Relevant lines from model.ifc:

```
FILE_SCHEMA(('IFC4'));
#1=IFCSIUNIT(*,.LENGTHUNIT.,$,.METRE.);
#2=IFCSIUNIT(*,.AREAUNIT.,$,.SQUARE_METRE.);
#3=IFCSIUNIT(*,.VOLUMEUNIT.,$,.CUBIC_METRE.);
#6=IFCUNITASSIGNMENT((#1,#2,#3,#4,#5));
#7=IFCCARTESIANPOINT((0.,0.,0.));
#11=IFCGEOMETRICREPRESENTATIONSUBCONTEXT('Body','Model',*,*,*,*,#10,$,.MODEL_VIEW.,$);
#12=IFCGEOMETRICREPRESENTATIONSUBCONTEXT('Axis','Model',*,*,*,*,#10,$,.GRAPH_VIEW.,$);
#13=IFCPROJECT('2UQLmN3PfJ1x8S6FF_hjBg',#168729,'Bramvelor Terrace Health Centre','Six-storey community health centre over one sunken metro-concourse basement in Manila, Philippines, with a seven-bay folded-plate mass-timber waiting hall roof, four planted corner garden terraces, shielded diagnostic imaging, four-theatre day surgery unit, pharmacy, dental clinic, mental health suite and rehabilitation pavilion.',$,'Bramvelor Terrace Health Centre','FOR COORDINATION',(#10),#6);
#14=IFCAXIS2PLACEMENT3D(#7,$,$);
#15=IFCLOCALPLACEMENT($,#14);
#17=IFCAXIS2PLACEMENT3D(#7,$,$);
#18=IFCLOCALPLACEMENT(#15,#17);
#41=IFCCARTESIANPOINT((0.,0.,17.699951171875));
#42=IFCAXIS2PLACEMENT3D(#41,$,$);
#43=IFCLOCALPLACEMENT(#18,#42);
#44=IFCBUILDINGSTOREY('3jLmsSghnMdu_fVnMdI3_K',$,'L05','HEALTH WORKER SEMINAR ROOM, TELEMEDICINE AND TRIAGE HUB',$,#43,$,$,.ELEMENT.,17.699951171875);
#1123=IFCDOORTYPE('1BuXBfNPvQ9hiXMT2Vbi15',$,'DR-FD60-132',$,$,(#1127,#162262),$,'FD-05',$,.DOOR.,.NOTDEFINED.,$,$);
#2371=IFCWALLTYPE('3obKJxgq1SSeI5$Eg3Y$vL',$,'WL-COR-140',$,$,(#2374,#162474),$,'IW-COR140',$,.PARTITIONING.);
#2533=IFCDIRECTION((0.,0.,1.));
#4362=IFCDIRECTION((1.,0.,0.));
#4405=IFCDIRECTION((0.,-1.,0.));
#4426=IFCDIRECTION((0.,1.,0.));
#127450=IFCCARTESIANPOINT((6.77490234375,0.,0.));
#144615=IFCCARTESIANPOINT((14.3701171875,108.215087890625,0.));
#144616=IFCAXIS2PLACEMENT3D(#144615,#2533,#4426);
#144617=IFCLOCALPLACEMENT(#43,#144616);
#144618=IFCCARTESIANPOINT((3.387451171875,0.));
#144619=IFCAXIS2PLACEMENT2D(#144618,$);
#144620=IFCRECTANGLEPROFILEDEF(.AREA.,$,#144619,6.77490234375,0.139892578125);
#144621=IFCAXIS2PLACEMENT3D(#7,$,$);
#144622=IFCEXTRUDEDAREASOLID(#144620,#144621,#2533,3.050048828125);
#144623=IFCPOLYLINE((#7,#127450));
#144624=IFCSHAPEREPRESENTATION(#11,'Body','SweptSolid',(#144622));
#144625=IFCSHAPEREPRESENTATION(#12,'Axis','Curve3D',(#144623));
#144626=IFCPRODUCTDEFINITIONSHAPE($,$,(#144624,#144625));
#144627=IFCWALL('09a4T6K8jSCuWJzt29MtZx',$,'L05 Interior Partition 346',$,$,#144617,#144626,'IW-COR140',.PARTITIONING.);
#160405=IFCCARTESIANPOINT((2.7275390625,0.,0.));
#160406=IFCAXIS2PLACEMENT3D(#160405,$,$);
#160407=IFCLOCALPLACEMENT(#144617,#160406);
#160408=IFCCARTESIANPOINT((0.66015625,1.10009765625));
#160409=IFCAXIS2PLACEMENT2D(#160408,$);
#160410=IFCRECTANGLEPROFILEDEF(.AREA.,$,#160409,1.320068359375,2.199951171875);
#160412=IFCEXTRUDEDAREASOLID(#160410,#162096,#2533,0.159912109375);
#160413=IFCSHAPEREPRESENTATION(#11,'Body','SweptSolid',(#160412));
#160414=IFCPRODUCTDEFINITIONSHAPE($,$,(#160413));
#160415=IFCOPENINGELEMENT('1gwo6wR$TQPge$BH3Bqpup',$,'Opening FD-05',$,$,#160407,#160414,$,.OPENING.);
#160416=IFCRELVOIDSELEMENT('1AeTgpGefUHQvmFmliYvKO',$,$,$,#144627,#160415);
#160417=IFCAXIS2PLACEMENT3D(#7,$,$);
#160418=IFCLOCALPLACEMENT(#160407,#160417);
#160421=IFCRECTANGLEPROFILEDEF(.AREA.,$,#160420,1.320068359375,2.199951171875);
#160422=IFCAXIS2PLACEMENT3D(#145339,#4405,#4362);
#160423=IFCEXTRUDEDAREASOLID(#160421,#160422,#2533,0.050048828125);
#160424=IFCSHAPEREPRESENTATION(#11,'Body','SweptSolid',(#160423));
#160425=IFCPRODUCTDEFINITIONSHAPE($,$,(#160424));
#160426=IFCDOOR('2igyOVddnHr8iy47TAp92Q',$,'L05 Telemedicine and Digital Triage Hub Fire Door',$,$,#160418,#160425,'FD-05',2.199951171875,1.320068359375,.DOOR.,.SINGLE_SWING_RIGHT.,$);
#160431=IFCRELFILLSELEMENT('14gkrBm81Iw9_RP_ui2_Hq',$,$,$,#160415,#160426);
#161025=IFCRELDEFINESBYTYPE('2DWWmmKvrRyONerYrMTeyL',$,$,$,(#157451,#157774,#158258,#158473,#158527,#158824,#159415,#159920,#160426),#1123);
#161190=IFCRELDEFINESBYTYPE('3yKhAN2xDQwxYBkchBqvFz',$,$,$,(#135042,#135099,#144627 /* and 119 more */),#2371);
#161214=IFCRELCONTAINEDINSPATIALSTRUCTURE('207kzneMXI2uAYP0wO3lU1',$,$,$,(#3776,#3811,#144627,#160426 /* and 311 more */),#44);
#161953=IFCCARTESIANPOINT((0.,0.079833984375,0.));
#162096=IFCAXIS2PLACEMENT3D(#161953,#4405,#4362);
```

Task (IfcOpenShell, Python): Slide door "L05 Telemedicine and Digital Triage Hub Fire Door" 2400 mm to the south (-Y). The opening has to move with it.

```python
import ifcopenshell
import ifcopenshell.api.geometry
import ifcopenshell.util.placement

model = ifcopenshell.open("model.ifc")

door = model.by_guid("2igyOVddnHr8iy47TAp92Q")
opening = door.FillsVoids[0].RelatingOpeningElement
wall = opening.VoidsElements[0].RelatingBuildingElement

wall_matrix = ifcopenshell.util.placement.get_local_placement(wall.ObjectPlacement)
shift = wall_matrix[:3, 0] * -2.4
before = ifcopenshell.util.placement.get_local_placement(door.ObjectPlacement)[:3, 3].copy()

# The door is placed relative to its opening, so it follows when the opening moves.
matrix = ifcopenshell.util.placement.get_local_placement(opening.ObjectPlacement)
matrix[:3, 3] += shift
ifcopenshell.api.geometry.edit_object_placement(
    model, product=opening, matrix=matrix, is_si=False, should_transform_children=True
)

after = ifcopenshell.util.placement.get_local_placement(door.ObjectPlacement)[:3, 3]
print("door moved by", (after - before).round(3) + 0.0)

model.write("model_edited.ifc")
```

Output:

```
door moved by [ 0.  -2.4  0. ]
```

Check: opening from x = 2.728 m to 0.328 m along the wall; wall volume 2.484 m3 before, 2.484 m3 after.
